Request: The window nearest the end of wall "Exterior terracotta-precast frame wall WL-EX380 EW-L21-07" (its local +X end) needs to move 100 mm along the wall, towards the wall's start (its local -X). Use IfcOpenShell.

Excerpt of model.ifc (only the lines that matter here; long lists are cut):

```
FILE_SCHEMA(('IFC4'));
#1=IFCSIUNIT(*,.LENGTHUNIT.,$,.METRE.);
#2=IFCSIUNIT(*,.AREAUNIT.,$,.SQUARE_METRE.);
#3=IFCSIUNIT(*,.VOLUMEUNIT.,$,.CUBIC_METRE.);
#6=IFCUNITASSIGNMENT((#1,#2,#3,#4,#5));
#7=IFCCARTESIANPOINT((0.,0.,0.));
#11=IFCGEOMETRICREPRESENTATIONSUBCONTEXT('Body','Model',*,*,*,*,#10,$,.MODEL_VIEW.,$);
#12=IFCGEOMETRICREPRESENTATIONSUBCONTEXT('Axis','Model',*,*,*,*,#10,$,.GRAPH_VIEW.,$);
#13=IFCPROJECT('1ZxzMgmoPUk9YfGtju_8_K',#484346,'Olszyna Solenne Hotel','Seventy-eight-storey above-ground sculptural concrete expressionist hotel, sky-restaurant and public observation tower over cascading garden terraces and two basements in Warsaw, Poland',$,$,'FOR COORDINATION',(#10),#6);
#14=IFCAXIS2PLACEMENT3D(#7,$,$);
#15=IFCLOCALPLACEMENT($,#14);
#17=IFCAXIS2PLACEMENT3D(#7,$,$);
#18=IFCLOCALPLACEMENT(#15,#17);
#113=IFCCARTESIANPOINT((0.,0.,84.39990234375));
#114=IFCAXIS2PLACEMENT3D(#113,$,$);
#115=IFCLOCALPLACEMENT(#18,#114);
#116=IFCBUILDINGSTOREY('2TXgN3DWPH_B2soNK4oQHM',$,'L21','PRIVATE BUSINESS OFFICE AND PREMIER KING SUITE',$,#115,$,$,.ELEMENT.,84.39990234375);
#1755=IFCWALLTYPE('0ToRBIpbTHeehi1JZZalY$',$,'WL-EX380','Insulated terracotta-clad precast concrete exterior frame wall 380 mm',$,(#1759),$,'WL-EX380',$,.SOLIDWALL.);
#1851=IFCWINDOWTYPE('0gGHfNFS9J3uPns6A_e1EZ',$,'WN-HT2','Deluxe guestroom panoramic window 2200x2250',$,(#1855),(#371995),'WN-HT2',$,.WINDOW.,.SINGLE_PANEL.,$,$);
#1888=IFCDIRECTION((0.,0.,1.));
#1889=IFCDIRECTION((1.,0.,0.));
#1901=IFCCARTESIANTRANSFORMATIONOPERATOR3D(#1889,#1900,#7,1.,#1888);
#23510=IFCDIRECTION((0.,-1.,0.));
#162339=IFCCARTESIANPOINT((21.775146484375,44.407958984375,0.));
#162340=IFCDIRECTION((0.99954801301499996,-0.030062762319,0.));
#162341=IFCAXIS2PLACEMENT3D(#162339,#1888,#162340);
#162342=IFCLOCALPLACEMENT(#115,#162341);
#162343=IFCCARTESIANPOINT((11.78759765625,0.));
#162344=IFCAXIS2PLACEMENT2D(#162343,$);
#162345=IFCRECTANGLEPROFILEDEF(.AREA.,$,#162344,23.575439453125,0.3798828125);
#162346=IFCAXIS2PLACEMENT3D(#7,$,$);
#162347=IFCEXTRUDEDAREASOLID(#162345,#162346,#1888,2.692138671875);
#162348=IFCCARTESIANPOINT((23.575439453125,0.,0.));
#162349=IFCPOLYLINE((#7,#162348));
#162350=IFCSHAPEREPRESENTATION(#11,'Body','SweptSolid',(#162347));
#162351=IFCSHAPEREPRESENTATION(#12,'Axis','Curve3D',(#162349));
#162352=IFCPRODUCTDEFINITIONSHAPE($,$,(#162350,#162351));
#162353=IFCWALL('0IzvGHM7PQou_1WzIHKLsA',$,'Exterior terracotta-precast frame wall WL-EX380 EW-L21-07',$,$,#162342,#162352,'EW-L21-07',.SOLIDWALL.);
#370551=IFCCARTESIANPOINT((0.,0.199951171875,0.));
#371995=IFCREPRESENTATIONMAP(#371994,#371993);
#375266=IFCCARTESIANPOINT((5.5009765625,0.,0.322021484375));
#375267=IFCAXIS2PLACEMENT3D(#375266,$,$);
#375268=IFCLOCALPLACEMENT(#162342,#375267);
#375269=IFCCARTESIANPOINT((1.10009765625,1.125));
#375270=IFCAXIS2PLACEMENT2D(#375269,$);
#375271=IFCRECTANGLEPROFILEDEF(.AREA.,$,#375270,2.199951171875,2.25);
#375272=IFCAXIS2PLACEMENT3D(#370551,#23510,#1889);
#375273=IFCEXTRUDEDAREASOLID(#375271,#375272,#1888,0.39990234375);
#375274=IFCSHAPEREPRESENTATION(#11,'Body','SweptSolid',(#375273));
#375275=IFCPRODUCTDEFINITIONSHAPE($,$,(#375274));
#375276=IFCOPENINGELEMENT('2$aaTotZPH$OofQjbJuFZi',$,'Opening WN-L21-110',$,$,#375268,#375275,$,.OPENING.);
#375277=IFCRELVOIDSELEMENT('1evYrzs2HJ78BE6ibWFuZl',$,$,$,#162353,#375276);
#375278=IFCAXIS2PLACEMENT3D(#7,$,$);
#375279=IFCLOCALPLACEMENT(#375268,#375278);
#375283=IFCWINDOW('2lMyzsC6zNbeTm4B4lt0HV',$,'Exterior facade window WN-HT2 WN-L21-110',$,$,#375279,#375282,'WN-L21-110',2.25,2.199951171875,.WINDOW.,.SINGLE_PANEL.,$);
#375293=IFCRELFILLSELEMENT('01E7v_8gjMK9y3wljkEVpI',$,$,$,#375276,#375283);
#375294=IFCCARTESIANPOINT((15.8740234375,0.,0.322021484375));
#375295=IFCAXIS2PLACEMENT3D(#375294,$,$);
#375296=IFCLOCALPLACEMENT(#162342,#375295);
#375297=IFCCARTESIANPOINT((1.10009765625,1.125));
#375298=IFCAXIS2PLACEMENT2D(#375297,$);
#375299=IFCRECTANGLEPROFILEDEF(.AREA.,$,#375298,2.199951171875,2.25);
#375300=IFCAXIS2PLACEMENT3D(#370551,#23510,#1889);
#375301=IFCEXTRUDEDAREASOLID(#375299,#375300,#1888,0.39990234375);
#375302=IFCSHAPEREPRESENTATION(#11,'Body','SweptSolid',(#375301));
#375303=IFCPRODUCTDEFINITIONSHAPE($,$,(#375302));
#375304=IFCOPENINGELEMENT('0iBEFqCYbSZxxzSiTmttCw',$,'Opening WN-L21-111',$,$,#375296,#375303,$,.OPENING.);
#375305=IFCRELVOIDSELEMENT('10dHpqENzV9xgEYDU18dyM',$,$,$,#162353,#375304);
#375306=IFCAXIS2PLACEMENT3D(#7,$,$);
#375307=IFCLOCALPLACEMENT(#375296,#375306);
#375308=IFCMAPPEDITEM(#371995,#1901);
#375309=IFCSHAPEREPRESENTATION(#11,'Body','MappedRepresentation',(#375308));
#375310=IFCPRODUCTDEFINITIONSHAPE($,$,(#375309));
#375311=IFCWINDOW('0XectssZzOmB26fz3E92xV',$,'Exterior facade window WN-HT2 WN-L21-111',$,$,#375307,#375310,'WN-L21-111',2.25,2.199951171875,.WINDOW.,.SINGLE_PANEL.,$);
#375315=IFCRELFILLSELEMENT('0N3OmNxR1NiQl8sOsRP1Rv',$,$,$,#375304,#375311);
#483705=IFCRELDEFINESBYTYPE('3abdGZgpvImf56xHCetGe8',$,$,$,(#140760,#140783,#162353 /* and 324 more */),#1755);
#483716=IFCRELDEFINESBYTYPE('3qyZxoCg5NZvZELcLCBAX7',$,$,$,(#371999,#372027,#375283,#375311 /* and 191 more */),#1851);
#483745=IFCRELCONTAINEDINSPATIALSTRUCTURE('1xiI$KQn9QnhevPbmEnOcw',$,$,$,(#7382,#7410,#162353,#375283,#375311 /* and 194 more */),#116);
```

```python
import ifcopenshell
import ifcopenshell.api.geometry
import ifcopenshell.util.placement

model = ifcopenshell.open("model.ifc")

window = model.by_guid("0XectssZzOmB26fz3E92xV")
opening = window.FillsVoids[0].RelatingOpeningElement
wall = opening.VoidsElements[0].RelatingBuildingElement

wall_matrix = ifcopenshell.util.placement.get_local_placement(wall.ObjectPlacement)
shift = wall_matrix[:3, 0] * -0.1
before = ifcopenshell.util.placement.get_local_placement(window.ObjectPlacement)[:3, 3].copy()

# The window is placed relative to its opening, so it follows when the opening moves.
matrix = ifcopenshell.util.placement.get_local_placement(opening.ObjectPlacement)
matrix[:3, 3] += shift
ifcopenshell.api.geometry.edit_object_placement(
    model, product=opening, matrix=matrix, is_si=False, should_transform_children=True
)

after = ifcopenshell.util.placement.get_local_placement(window.ObjectPlacement)[:3, 3]
print("window moved by", (after - before).round(3) + 0.0)

model.write("model_edited.ifc")
```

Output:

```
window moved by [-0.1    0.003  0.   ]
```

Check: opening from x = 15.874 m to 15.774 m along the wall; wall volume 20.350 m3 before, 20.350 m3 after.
